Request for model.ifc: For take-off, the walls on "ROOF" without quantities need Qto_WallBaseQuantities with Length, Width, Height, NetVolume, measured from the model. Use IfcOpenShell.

First a look at what the model holds.

```python
import ifcopenshell
import ifcopenshell.util.element
import ifcopenshell.util.unit

model = ifcopenshell.open("model.ifc")
print(model.schema)
for unit_type in ("LENGTHUNIT", "AREAUNIT", "VOLUMEUNIT"):
    print(unit_type, ifcopenshell.util.unit.calculate_unit_scale(model, unit_type))
storey = next(s for s in model.by_type("IfcBuildingStorey") if s.Name == "ROOF")
walls = [e for e in ifcopenshell.util.element.get_decomposition(storey) if e.is_a("IfcWall")]
for e in sorted(walls, key=lambda e: e.id()):
    print(e.id(), e.is_a(), e.Name, list(ifcopenshell.util.element.get_psets(e, qtos_only=True)), sep=" | ")
```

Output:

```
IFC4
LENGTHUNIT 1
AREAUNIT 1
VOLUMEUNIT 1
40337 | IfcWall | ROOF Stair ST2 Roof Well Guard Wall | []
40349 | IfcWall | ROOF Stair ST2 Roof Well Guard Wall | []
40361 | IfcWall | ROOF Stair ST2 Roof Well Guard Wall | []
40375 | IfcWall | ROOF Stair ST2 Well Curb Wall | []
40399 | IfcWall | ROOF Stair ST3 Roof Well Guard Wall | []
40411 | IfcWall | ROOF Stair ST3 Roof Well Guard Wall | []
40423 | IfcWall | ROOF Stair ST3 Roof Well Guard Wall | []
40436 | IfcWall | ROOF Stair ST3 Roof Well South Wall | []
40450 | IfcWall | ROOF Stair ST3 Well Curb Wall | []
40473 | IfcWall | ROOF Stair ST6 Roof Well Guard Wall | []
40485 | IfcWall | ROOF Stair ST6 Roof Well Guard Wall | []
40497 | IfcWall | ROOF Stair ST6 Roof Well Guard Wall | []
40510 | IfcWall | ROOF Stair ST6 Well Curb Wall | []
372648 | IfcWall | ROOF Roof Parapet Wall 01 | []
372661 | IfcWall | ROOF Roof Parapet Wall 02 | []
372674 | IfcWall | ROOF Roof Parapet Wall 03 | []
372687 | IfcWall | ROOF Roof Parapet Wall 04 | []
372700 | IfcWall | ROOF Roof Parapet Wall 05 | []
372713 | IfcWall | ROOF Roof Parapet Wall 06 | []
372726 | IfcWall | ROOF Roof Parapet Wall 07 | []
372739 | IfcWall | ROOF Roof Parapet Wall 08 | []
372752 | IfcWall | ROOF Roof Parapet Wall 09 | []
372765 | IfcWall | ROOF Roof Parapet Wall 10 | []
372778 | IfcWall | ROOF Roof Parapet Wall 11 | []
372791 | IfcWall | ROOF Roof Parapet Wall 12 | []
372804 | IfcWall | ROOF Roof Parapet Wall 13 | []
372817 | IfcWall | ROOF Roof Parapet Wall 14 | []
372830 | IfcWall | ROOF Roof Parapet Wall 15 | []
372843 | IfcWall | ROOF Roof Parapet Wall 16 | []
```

```python
import ifcopenshell
import ifcopenshell.api.pset
import ifcopenshell.geom
import ifcopenshell.util.element
import ifcopenshell.util.shape
import ifcopenshell.util.unit

model = ifcopenshell.open("model.ifc")
unit_scale = ifcopenshell.util.unit.calculate_unit_scale(model)
volume_scale = ifcopenshell.util.unit.calculate_unit_scale(model, "VOLUMEUNIT")
settings = ifcopenshell.geom.settings()

storey = next(s for s in model.by_type("IfcBuildingStorey") if s.Name == "ROOF")
walls = [e for e in ifcopenshell.util.element.get_decomposition(storey) if e.is_a("IfcWall")]

for e in sorted(walls, key=lambda e: e.id()):
    if ifcopenshell.util.element.get_psets(e, qtos_only=True, should_inherit=False):
        continue
    # Geometry comes back in metres, in the element's own axes.
    shape = ifcopenshell.geom.create_shape(settings, e)
    values = {
        "Length": ifcopenshell.util.shape.get_x(shape.geometry) / unit_scale,
        "Width": ifcopenshell.util.shape.get_y(shape.geometry) / unit_scale,
        "Height": ifcopenshell.util.shape.get_z(shape.geometry) / unit_scale,
        "NetVolume": ifcopenshell.util.shape.get_volume(shape.geometry) / volume_scale,
    }
    qto = ifcopenshell.api.pset.add_qto(model, product=e, name="Qto_WallBaseQuantities")
    ifcopenshell.api.pset.edit_qto(model, qto=qto, properties=values)
    print(e.id(), {k: round(v, 3) for k, v in values.items()})

model.write("model_edited.ifc")
```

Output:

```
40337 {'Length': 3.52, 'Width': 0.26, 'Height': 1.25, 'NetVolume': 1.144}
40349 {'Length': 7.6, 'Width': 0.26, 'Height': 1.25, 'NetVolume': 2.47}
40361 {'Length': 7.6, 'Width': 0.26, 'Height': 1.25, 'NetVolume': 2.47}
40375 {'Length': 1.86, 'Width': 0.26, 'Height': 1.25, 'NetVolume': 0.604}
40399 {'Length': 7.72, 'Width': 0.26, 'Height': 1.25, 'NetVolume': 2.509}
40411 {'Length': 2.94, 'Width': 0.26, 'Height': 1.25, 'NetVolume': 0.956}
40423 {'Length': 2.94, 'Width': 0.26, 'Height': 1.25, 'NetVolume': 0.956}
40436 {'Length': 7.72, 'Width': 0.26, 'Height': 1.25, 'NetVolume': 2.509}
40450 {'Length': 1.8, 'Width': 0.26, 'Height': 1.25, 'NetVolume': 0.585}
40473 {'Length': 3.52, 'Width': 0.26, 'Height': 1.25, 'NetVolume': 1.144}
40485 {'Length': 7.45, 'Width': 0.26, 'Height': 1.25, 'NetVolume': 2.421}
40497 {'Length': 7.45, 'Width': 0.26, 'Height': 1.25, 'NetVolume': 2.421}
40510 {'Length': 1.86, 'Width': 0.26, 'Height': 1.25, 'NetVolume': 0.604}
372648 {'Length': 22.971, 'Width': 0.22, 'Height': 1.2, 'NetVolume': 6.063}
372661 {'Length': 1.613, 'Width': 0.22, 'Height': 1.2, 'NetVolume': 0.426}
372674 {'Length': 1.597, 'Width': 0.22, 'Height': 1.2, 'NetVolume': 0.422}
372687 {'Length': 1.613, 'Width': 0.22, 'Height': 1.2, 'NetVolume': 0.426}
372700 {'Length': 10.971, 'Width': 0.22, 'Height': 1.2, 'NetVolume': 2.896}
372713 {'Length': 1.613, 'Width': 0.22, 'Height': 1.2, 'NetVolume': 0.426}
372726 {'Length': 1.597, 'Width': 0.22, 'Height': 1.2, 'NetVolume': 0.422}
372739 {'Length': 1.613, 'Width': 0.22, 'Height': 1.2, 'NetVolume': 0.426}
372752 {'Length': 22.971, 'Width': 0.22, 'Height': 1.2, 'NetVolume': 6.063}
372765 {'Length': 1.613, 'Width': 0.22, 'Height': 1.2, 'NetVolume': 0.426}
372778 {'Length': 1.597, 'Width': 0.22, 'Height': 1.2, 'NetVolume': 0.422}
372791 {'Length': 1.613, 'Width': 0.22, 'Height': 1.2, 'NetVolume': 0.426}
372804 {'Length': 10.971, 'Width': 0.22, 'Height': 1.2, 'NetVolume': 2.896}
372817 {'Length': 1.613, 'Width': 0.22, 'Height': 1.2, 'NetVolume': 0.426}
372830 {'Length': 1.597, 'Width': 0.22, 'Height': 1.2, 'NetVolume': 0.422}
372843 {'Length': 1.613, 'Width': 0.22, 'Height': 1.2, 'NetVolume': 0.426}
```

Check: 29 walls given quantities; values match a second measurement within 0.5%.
